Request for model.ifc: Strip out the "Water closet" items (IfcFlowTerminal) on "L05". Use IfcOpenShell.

First a look at what the model holds.

```python
import ifcopenshell
import ifcopenshell.util.element

model = ifcopenshell.open("model.ifc")
print(model.schema)
storey = next(s for s in model.by_type("IfcBuildingStorey") if s.Name == "L05")
terminals = [e for e in ifcopenshell.util.element.get_decomposition(storey) if e.is_a("IfcFlowTerminal")]
seen = {}
for e in terminals:
    element_type = ifcopenshell.util.element.get_type(e)
    name = element_type.Name if element_type not in (None, e) else None
    seen[name] = seen.get(name, 0) + 1
for name, count in sorted(seen.items(), key=str):
    print(count, "x", name)
```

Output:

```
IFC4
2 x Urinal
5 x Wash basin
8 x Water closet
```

```python
import ifcopenshell
import ifcopenshell.api.root
import ifcopenshell.util.element

model = ifcopenshell.open("model.ifc")

storey = next(s for s in model.by_type("IfcBuildingStorey") if s.Name == "L05")
terminals = [e for e in ifcopenshell.util.element.get_decomposition(storey) if e.is_a("IfcFlowTerminal")]
targets = [e for e in terminals if (t := ifcopenshell.util.element.get_type(e)) not in (None, e) and t.Name == "Water closet"]

for e in targets:
    ifcopenshell.api.root.remove_product(model, product=e)
print(len(targets), "removed")

model.write("model_edited.ifc")
```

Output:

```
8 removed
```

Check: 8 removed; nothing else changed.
